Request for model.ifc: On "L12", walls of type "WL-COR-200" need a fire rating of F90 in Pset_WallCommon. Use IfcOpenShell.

First a look at what the model holds.

```python
import ifcopenshell
import ifcopenshell.util.element

model = ifcopenshell.open("model.ifc")
print(model.schema)
storey = next(s for s in model.by_type("IfcBuildingStorey") if s.Name == "L12")
walls = [e for e in ifcopenshell.util.element.get_decomposition(storey) if e.is_a("IfcWall")]
seen = {}
for e in walls:
    element_type = ifcopenshell.util.element.get_type(e)
    key = (element_type.Name if element_type != e and element_type else None, ifcopenshell.util.element.get_pset(e, "Pset_WallCommon", "FireRating"))
    seen[key] = seen.get(key, 0) + 1
for (name, value), count in sorted(seen.items(), key=str):
    print(count, "x", name, "|", value)
```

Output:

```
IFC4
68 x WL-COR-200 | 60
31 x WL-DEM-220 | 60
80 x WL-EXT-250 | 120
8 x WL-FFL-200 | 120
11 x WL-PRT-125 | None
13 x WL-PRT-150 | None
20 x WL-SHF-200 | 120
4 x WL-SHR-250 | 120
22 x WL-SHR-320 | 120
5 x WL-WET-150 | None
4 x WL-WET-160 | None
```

```python
import ifcopenshell
import ifcopenshell.api.pset
import ifcopenshell.util.element

model = ifcopenshell.open("model.ifc")

storey = next(s for s in model.by_type("IfcBuildingStorey") if s.Name == "L12")
walls = [e for e in ifcopenshell.util.element.get_decomposition(storey) if e.is_a("IfcWall")]

count = 0
for e in walls:
    element_type = ifcopenshell.util.element.get_type(e)
    if element_type in (None, e) or element_type.Name != "WL-COR-200":
        continue
    # add_pset returns the element's existing set when there is one.
    pset = ifcopenshell.api.pset.add_pset(model, product=e, name="Pset_WallCommon")
    ifcopenshell.api.pset.edit_pset(model, pset=pset, properties={"FireRating": "F90"})
    count += 1

print(count, "walls updated")

model.write("model_updated.ifc")
```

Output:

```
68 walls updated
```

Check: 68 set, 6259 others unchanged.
